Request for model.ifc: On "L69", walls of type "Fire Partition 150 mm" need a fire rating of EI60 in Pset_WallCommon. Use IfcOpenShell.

First a look at what the model holds.

```python
import ifcopenshell
import ifcopenshell.util.element

model = ifcopenshell.open("model.ifc")
print(model.schema)
storey = next(s for s in model.by_type("IfcBuildingStorey") if s.Name == "L69")
walls = [e for e in ifcopenshell.util.element.get_decomposition(storey) if e.is_a("IfcWall")]
seen = {}
for e in walls:
    element_type = ifcopenshell.util.element.get_type(e)
    key = (element_type.Name if element_type != e and element_type else None, ifcopenshell.util.element.get_pset(e, "Pset_WallCommon", "FireRating"))
    seen[key] = seen.get(key, 0) + 1
for (name, value), count in sorted(seen.items(), key=str):
    print(count, "x", name, "|", value)
```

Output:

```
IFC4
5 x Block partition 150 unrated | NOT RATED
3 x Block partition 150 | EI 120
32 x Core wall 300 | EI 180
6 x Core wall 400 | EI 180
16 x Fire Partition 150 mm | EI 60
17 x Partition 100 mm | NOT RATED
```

```python
import ifcopenshell
import ifcopenshell.api.pset
import ifcopenshell.util.element

model = ifcopenshell.open("model.ifc")

storey = next(s for s in model.by_type("IfcBuildingStorey") if s.Name == "L69")
walls = [e for e in ifcopenshell.util.element.get_decomposition(storey) if e.is_a("IfcWall")]

count = 0
for e in walls:
    element_type = ifcopenshell.util.element.get_type(e)
    if element_type in (None, e) or element_type.Name != "Fire Partition 150 mm":
        continue
    found = ifcopenshell.util.element.get_pset(e, "Pset_WallCommon", should_inherit=False)
    if found:
        pset = model.by_id(found["id"])
        if len(ifcopenshell.util.element.get_elements_by_pset(pset)) > 1:
            pset = ifcopenshell.api.pset.unshare_pset(model, products=[e], pset=pset)[0]
    else:
        pset = ifcopenshell.api.pset.add_pset(model, product=e, name="Pset_WallCommon")
    ifcopenshell.api.pset.edit_pset(model, pset=pset, properties={"FireRating": "EI60"})
    count += 1

print(count, "walls updated")

model.write("model_updated.ifc")
```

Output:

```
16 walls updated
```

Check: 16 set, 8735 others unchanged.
